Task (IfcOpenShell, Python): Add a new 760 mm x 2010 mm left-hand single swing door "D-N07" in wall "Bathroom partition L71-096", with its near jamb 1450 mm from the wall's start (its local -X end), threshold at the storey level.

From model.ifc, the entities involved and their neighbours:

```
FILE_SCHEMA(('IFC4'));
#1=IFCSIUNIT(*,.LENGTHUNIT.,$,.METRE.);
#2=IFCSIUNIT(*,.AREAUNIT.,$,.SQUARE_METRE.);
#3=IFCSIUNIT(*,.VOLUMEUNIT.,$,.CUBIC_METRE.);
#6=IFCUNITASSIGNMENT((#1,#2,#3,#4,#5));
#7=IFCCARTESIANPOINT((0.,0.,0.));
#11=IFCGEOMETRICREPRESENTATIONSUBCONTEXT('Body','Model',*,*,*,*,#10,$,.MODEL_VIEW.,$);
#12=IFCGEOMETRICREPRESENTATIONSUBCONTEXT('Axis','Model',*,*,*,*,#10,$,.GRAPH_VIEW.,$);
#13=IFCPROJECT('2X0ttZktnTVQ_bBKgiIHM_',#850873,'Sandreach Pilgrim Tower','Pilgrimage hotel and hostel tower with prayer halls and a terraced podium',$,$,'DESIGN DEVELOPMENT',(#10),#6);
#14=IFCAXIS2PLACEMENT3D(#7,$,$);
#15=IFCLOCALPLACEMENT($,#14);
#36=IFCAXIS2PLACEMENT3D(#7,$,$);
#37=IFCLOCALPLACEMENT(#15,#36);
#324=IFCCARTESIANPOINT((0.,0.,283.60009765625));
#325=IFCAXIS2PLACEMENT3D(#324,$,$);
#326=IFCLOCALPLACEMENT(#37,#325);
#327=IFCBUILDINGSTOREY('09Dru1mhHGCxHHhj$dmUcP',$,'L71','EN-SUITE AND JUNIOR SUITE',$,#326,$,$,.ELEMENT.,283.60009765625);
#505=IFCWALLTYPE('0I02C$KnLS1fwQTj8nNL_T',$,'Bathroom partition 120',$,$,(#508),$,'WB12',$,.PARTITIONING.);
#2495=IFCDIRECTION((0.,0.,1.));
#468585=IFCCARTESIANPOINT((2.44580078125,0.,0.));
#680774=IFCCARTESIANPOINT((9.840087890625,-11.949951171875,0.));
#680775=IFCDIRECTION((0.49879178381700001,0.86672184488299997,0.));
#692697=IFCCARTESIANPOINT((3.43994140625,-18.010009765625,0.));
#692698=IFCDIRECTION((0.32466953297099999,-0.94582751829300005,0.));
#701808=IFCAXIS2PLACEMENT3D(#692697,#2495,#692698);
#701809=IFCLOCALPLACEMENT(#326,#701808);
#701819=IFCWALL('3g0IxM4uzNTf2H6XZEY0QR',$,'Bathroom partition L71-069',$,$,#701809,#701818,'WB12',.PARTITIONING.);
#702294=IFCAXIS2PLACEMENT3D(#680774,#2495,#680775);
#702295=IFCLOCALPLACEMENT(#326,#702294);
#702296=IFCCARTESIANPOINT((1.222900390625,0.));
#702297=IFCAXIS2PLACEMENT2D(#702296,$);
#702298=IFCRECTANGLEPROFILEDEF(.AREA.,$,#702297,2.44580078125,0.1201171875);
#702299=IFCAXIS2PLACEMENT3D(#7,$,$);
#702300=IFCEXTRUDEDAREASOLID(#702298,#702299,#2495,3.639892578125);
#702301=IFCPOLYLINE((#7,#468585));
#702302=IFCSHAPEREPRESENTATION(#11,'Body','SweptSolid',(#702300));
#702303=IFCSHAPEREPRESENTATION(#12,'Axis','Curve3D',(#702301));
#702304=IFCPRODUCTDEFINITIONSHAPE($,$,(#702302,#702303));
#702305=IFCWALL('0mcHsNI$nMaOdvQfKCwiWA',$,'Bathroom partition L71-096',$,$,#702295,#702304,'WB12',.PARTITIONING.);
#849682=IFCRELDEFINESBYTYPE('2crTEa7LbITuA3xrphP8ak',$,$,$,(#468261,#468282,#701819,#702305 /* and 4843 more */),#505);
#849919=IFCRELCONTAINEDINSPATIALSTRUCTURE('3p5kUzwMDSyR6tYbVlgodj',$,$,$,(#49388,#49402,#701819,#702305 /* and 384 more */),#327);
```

```python
import numpy as np
import ifcopenshell
import ifcopenshell.api.feature
import ifcopenshell.api.geometry
import ifcopenshell.api.root
import ifcopenshell.api.spatial
import ifcopenshell.geom
import ifcopenshell.util.element
import ifcopenshell.util.placement
import ifcopenshell.util.representation
import ifcopenshell.util.shape
import ifcopenshell.util.unit

model = ifcopenshell.open("model.ifc")
unit_scale = ifcopenshell.util.unit.calculate_unit_scale(model)
settings = ifcopenshell.geom.settings()


def volume(element):
    """Net volume in cubic metres, openings subtracted."""
    shape = ifcopenshell.geom.create_shape(settings, element)
    return ifcopenshell.util.shape.get_volume(shape.geometry)


wall = model.by_guid("0mcHsNI$nMaOdvQfKCwiWA")
storey = ifcopenshell.util.element.get_container(wall, ifc_class="IfcBuildingStorey")
context = ifcopenshell.util.representation.get_context(model, "Model", "Body", "MODEL_VIEW")
before = volume(wall)

width, height, from_end, sill = 0.76, 2.01, 1.45, 0.0  # metres

# The wall runs along its own X axis, and the end named is its -X end.
wall_shape = ifcopenshell.geom.create_shape(settings, wall)
x, y, z = ifcopenshell.util.shape.get_vertices(wall_shape.geometry).T
start = x.min() + from_end
face, thickness = float(y.min()), float(y.max() - y.min())
wall_matrix = ifcopenshell.util.placement.get_local_placement(wall.ObjectPlacement)
level = ifcopenshell.util.placement.get_local_placement(storey.ObjectPlacement)[2, 3]


def in_wall(x, y):
    """Placement at x, y metres in the wall's axes, at sill height."""
    matrix = wall_matrix.copy()
    matrix[:, 3] = wall_matrix @ np.array([x / unit_scale, y / unit_scale, 0.0, 1.0])
    matrix[2, 3] = level + sill / unit_scale
    return matrix


# Opening: a box that overshoots both wall faces by 50 mm.
opening = ifcopenshell.api.root.create_entity(model, ifc_class="IfcOpeningElement", predefined_type="OPENING")
box = ifcopenshell.api.geometry.add_wall_representation(
    model, context=context, length=width, height=height, thickness=thickness + 0.1
)
ifcopenshell.api.geometry.assign_representation(model, product=opening, representation=box)
ifcopenshell.api.geometry.edit_object_placement(model, product=opening, matrix=in_wall(start, face - 0.05), is_si=False)
ifcopenshell.api.feature.add_feature(model, feature=opening, element=wall)

door = ifcopenshell.api.root.create_entity(model, ifc_class="IfcDoor", name="D-N07", predefined_type="DOOR")
door.OverallWidth, door.OverallHeight = width / unit_scale, height / unit_scale
door.OperationType = "SINGLE_SWING_LEFT"
body = ifcopenshell.api.geometry.add_door_representation(
    model,
    context=context,
    overall_width=door.OverallWidth,
    overall_height=door.OverallHeight,
    operation_type="SINGLE_SWING_LEFT",
    lining_properties={"LiningDepth": thickness / unit_scale, "ThresholdDepth": thickness / unit_scale},
)
ifcopenshell.api.geometry.assign_representation(model, product=door, representation=body)
ifcopenshell.api.spatial.assign_container(model, products=[door], relating_structure=storey)
ifcopenshell.api.feature.add_filling(model, opening=opening, element=door)

# The lining spans the wall, so the door starts at the wall face.
ifcopenshell.api.geometry.edit_object_placement(model, product=door, matrix=in_wall(start, face), is_si=False)

after = volume(wall)

print(f"wall volume {before:.3f} -> {after:.3f} m3")

model.write("model_rev.ifc")
```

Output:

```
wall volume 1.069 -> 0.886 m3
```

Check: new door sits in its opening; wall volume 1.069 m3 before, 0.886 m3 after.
